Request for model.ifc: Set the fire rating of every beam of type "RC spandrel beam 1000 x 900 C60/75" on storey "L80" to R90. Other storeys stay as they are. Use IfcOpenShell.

First a look at what the model holds.

```python
import ifcopenshell
import ifcopenshell.util.element

model = ifcopenshell.open("model.ifc")
print(model.schema)
storey = next(s for s in model.by_type("IfcBuildingStorey") if s.Name == "L80")
beams = [e for e in ifcopenshell.util.element.get_decomposition(storey) if e.is_a("IfcBeam")]
seen = {}
for e in beams:
    element_type = ifcopenshell.util.element.get_type(e)
    key = (element_type.Name if element_type != e and element_type else None, ifcopenshell.util.element.get_pset(e, "Pset_BeamCommon", "FireRating"))
    seen[key] = seen.get(key, 0) + 1
for (name, value), count in sorted(seen.items(), key=str):
    print(count, "x", name, "|", value)
```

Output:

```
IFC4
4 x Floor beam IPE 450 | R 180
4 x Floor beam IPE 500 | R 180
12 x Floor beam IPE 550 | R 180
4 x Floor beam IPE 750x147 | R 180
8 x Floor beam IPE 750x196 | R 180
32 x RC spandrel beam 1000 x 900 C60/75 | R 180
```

```python
import ifcopenshell
import ifcopenshell.api.pset
import ifcopenshell.util.element

model = ifcopenshell.open("model.ifc")

storey = next(s for s in model.by_type("IfcBuildingStorey") if s.Name == "L80")
beams = [e for e in ifcopenshell.util.element.get_decomposition(storey) if e.is_a("IfcBeam")]

count = 0
for e in beams:
    element_type = ifcopenshell.util.element.get_type(e)
    if element_type in (None, e) or element_type.Name != "RC spandrel beam 1000 x 900 C60/75":
        continue
    found = ifcopenshell.util.element.get_pset(e, "Pset_BeamCommon", should_inherit=False)
    if found:
        pset = model.by_id(found["id"])
        if len(ifcopenshell.util.element.get_elements_by_pset(pset)) > 1:
            pset = ifcopenshell.api.pset.unshare_pset(model, products=[e], pset=pset)[0]
    else:
        pset = ifcopenshell.api.pset.add_pset(model, product=e, name="Pset_BeamCommon")
    ifcopenshell.api.pset.edit_pset(model, pset=pset, properties={"FireRating": "R90"})
    count += 1

print(count, "beams updated")

model.write("model_edited.ifc")
```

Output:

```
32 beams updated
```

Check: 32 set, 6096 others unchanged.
